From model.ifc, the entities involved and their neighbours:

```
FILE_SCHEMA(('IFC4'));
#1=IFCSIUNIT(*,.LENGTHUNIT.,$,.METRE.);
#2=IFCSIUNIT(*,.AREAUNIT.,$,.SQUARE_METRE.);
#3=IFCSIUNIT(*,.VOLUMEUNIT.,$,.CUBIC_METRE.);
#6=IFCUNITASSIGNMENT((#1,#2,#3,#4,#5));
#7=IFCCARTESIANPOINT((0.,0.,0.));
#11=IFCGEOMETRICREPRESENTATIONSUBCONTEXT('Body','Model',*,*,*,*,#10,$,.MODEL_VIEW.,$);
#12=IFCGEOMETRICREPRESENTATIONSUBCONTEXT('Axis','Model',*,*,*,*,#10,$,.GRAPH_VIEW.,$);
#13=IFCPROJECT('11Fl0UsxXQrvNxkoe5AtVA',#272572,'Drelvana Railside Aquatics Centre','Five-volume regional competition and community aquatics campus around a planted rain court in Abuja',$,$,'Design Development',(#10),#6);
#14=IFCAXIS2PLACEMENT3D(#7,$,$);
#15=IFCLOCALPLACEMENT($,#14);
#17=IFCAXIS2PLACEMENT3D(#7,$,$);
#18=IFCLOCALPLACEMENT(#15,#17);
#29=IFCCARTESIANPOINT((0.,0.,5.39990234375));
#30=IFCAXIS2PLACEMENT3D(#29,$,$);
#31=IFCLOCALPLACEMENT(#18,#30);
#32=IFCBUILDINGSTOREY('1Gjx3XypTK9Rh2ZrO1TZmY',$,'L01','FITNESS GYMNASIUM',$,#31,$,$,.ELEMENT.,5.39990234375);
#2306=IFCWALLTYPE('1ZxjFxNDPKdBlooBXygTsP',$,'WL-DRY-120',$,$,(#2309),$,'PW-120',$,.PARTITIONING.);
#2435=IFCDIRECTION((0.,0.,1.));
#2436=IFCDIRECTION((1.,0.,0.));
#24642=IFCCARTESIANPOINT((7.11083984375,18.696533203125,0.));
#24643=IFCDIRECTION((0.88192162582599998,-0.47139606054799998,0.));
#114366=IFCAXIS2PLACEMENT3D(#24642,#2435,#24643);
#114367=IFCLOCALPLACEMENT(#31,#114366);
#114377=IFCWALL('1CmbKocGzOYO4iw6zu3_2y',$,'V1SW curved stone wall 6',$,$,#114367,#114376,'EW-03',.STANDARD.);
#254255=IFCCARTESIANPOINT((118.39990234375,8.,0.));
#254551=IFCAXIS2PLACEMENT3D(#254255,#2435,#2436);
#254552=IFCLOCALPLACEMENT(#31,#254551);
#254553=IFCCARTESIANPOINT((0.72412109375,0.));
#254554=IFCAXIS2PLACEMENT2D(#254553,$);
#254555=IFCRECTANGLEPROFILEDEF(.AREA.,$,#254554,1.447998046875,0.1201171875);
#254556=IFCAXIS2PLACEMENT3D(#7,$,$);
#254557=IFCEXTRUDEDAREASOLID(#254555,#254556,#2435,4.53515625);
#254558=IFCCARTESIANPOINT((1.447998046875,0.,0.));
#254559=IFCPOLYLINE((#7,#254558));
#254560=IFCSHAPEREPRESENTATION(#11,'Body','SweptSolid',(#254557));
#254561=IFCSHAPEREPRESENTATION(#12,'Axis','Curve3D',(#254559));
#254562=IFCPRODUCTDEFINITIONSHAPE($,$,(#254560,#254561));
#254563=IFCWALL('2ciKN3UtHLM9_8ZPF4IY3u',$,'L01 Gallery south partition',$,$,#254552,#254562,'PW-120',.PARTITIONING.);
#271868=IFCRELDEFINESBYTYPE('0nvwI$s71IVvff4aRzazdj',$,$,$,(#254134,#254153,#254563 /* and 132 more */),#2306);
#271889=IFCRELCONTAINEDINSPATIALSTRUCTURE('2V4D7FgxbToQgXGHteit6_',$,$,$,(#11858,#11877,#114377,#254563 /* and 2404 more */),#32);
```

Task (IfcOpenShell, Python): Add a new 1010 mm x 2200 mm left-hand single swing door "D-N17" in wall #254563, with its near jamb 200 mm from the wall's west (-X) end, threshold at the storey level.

```python
import numpy as np
import ifcopenshell
import ifcopenshell.api.feature
import ifcopenshell.api.geometry
import ifcopenshell.api.root
import ifcopenshell.api.spatial
import ifcopenshell.geom
import ifcopenshell.util.element
import ifcopenshell.util.placement
import ifcopenshell.util.representation
import ifcopenshell.util.shape
import ifcopenshell.util.unit

model = ifcopenshell.open("model.ifc")
unit_scale = ifcopenshell.util.unit.calculate_unit_scale(model)
settings = ifcopenshell.geom.settings()


def volume(element):
    """Net volume in cubic metres, openings subtracted."""
    shape = ifcopenshell.geom.create_shape(settings, element)
    return ifcopenshell.util.shape.get_volume(shape.geometry)


wall = model.by_guid("2ciKN3UtHLM9_8ZPF4IY3u")
storey = ifcopenshell.util.element.get_container(wall, ifc_class="IfcBuildingStorey")
context = ifcopenshell.util.representation.get_context(model, "Model", "Body", "MODEL_VIEW")
before = volume(wall)

width, height, from_end, sill = 1.01, 2.2, 0.2, 0.0  # metres

# The wall runs along its own X axis, and the end named is its -X end.
wall_shape = ifcopenshell.geom.create_shape(settings, wall)
x, y, z = ifcopenshell.util.shape.get_vertices(wall_shape.geometry).T
start = x.min() + from_end
face, thickness = float(y.min()), float(y.max() - y.min())
wall_matrix = ifcopenshell.util.placement.get_local_placement(wall.ObjectPlacement)
level = ifcopenshell.util.placement.get_local_placement(storey.ObjectPlacement)[2, 3]


def in_wall(x, y):
    """Placement at x, y metres in the wall's axes, at sill height."""
    matrix = wall_matrix.copy()
    matrix[:, 3] = wall_matrix @ np.array([x / unit_scale, y / unit_scale, 0.0, 1.0])
    matrix[2, 3] = level + sill / unit_scale
    return matrix


# Opening: a box that overshoots both wall faces by 50 mm.
opening = ifcopenshell.api.root.create_entity(model, ifc_class="IfcOpeningElement", predefined_type="OPENING")
box = ifcopenshell.api.geometry.add_wall_representation(
    model, context=context, length=width, height=height, thickness=thickness + 0.1
)
ifcopenshell.api.geometry.assign_representation(model, product=opening, representation=box)
ifcopenshell.api.geometry.edit_object_placement(model, product=opening, matrix=in_wall(start, face - 0.05), is_si=False)
ifcopenshell.api.feature.add_feature(model, feature=opening, element=wall)

door = ifcopenshell.api.root.create_entity(model, ifc_class="IfcDoor", name="D-N17", predefined_type="DOOR")
door.OverallWidth, door.OverallHeight = width / unit_scale, height / unit_scale
door.OperationType = "SINGLE_SWING_LEFT"
body = ifcopenshell.api.geometry.add_door_representation(
    model,
    context=context,
    overall_width=door.OverallWidth,
    overall_height=door.OverallHeight,
    operation_type="SINGLE_SWING_LEFT",
    lining_properties={"LiningDepth": thickness / unit_scale, "ThresholdDepth": thickness / unit_scale},
)
ifcopenshell.api.geometry.assign_representation(model, product=door, representation=body)
ifcopenshell.api.spatial.assign_container(model, products=[door], relating_structure=storey)
ifcopenshell.api.feature.add_filling(model, opening=opening, element=door)

# The lining spans the wall, so the door starts at the wall face.
ifcopenshell.api.geometry.edit_object_placement(model, product=door, matrix=in_wall(start, face), is_si=False)

after = volume(wall)

print(f"wall volume {before:.3f} -> {after:.3f} m3")

model.write("model-out.ifc")
```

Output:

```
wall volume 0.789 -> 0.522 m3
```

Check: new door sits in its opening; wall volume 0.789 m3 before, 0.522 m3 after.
